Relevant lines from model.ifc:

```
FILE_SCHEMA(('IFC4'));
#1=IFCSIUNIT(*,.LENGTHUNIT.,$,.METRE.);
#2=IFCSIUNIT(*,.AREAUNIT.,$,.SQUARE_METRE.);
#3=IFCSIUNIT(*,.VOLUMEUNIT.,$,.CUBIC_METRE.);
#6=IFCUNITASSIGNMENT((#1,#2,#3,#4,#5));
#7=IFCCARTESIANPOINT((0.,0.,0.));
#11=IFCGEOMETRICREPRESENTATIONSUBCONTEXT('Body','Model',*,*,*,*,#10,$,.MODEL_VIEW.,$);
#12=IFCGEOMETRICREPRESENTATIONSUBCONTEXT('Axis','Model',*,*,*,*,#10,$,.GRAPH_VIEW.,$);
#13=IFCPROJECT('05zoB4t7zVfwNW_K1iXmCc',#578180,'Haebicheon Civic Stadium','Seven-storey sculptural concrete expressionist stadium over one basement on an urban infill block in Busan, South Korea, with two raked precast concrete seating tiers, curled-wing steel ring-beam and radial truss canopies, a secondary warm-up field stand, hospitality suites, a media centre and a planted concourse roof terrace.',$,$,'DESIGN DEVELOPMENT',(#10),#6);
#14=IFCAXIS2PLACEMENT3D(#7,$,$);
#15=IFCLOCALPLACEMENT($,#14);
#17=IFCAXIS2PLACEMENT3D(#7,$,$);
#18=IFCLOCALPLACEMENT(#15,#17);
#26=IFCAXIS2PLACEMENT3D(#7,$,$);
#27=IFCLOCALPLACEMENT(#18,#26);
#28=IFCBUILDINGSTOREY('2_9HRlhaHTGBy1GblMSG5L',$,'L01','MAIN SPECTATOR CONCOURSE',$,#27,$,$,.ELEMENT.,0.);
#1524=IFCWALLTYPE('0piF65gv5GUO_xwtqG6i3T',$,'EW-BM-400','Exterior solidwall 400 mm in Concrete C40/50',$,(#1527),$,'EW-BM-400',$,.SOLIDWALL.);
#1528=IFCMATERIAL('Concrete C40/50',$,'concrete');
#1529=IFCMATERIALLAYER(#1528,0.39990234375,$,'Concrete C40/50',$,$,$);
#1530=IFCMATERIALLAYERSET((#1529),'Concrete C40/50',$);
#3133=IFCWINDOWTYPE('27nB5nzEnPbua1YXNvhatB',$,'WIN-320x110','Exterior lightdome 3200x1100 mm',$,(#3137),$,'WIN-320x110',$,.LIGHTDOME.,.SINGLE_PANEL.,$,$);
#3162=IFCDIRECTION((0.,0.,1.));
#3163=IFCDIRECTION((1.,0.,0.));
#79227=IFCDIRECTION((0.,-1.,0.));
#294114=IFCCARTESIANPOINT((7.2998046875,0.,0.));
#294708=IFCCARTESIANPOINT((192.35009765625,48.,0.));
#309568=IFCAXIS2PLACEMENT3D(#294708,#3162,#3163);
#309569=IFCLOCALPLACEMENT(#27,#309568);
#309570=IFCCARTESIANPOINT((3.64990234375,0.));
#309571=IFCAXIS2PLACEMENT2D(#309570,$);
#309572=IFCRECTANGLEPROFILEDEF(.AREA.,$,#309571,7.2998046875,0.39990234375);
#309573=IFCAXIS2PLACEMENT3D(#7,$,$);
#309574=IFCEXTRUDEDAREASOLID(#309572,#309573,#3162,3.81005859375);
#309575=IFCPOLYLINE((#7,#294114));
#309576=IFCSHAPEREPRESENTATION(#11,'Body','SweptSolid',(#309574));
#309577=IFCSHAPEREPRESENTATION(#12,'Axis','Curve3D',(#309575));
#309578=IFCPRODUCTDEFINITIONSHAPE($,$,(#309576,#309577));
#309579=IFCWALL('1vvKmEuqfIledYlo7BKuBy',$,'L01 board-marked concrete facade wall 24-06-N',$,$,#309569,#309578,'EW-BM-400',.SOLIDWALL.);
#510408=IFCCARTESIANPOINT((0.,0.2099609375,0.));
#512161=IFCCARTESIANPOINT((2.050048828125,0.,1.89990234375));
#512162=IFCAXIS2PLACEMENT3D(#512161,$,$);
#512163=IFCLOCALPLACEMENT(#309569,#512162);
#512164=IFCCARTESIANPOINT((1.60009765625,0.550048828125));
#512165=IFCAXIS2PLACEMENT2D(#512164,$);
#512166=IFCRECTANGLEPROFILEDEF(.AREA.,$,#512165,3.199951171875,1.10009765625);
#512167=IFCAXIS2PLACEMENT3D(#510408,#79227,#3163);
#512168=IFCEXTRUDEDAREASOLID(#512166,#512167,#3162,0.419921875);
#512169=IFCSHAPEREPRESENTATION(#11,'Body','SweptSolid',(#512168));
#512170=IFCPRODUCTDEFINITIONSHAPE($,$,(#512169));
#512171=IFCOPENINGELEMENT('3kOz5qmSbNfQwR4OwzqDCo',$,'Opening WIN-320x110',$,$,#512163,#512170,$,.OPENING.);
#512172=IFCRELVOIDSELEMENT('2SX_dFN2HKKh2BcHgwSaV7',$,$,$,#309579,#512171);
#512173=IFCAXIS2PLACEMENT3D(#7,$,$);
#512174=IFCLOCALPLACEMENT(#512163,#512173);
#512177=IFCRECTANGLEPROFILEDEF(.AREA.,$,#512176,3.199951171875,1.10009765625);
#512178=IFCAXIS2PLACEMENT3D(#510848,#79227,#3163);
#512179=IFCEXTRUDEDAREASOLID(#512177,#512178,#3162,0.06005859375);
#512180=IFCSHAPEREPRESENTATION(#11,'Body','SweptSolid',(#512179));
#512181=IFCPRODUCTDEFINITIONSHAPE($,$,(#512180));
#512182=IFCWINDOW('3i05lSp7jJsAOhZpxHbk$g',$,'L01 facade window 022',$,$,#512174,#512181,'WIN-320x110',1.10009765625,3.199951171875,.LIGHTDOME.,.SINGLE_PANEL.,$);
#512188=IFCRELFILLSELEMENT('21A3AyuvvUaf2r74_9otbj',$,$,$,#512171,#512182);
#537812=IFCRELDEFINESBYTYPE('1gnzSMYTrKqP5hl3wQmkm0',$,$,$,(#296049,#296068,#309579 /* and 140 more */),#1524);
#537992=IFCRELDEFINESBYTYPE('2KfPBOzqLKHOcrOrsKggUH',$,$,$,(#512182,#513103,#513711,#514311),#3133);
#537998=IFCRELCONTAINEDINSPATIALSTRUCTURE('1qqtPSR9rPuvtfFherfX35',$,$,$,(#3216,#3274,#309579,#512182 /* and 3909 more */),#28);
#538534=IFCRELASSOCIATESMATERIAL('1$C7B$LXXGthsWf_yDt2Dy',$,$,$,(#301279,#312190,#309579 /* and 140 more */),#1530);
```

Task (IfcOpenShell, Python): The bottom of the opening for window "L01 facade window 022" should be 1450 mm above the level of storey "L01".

```python
import numpy as np
import ifcopenshell
import ifcopenshell.api.geometry
import ifcopenshell.geom
import ifcopenshell.util.element
import ifcopenshell.util.placement
import ifcopenshell.util.shape
import ifcopenshell.util.unit

model = ifcopenshell.open("model.ifc")
unit_scale = ifcopenshell.util.unit.calculate_unit_scale(model)

window = model.by_guid("3i05lSp7jJsAOhZpxHbk$g")
opening = window.FillsVoids[0].RelatingOpeningElement
storey = ifcopenshell.util.element.get_container(window, ifc_class="IfcBuildingStorey")
level = ifcopenshell.util.placement.get_local_placement(storey.ObjectPlacement)[2, 3]

# The opening's origin need not be at the sill, so measure its lowest point.
shape = ifcopenshell.geom.create_shape(ifcopenshell.geom.settings(), opening)
bottom = ifcopenshell.util.shape.get_shape_bottom_elevation(shape, shape.geometry) / unit_scale
dz = level + 1.45 - bottom

shift = np.array([0.0, 0.0, dz])
# The window is placed relative to its opening, so it follows when the opening moves.
matrix = ifcopenshell.util.placement.get_local_placement(opening.ObjectPlacement)
matrix[:3, 3] += shift
ifcopenshell.api.geometry.edit_object_placement(
    model, product=opening, matrix=matrix, is_si=False, should_transform_children=True
)

print(f"moved by {dz * unit_scale:+.3f} m")

model.write("model-out.ifc")
```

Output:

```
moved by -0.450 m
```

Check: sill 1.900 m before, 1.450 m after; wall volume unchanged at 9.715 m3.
